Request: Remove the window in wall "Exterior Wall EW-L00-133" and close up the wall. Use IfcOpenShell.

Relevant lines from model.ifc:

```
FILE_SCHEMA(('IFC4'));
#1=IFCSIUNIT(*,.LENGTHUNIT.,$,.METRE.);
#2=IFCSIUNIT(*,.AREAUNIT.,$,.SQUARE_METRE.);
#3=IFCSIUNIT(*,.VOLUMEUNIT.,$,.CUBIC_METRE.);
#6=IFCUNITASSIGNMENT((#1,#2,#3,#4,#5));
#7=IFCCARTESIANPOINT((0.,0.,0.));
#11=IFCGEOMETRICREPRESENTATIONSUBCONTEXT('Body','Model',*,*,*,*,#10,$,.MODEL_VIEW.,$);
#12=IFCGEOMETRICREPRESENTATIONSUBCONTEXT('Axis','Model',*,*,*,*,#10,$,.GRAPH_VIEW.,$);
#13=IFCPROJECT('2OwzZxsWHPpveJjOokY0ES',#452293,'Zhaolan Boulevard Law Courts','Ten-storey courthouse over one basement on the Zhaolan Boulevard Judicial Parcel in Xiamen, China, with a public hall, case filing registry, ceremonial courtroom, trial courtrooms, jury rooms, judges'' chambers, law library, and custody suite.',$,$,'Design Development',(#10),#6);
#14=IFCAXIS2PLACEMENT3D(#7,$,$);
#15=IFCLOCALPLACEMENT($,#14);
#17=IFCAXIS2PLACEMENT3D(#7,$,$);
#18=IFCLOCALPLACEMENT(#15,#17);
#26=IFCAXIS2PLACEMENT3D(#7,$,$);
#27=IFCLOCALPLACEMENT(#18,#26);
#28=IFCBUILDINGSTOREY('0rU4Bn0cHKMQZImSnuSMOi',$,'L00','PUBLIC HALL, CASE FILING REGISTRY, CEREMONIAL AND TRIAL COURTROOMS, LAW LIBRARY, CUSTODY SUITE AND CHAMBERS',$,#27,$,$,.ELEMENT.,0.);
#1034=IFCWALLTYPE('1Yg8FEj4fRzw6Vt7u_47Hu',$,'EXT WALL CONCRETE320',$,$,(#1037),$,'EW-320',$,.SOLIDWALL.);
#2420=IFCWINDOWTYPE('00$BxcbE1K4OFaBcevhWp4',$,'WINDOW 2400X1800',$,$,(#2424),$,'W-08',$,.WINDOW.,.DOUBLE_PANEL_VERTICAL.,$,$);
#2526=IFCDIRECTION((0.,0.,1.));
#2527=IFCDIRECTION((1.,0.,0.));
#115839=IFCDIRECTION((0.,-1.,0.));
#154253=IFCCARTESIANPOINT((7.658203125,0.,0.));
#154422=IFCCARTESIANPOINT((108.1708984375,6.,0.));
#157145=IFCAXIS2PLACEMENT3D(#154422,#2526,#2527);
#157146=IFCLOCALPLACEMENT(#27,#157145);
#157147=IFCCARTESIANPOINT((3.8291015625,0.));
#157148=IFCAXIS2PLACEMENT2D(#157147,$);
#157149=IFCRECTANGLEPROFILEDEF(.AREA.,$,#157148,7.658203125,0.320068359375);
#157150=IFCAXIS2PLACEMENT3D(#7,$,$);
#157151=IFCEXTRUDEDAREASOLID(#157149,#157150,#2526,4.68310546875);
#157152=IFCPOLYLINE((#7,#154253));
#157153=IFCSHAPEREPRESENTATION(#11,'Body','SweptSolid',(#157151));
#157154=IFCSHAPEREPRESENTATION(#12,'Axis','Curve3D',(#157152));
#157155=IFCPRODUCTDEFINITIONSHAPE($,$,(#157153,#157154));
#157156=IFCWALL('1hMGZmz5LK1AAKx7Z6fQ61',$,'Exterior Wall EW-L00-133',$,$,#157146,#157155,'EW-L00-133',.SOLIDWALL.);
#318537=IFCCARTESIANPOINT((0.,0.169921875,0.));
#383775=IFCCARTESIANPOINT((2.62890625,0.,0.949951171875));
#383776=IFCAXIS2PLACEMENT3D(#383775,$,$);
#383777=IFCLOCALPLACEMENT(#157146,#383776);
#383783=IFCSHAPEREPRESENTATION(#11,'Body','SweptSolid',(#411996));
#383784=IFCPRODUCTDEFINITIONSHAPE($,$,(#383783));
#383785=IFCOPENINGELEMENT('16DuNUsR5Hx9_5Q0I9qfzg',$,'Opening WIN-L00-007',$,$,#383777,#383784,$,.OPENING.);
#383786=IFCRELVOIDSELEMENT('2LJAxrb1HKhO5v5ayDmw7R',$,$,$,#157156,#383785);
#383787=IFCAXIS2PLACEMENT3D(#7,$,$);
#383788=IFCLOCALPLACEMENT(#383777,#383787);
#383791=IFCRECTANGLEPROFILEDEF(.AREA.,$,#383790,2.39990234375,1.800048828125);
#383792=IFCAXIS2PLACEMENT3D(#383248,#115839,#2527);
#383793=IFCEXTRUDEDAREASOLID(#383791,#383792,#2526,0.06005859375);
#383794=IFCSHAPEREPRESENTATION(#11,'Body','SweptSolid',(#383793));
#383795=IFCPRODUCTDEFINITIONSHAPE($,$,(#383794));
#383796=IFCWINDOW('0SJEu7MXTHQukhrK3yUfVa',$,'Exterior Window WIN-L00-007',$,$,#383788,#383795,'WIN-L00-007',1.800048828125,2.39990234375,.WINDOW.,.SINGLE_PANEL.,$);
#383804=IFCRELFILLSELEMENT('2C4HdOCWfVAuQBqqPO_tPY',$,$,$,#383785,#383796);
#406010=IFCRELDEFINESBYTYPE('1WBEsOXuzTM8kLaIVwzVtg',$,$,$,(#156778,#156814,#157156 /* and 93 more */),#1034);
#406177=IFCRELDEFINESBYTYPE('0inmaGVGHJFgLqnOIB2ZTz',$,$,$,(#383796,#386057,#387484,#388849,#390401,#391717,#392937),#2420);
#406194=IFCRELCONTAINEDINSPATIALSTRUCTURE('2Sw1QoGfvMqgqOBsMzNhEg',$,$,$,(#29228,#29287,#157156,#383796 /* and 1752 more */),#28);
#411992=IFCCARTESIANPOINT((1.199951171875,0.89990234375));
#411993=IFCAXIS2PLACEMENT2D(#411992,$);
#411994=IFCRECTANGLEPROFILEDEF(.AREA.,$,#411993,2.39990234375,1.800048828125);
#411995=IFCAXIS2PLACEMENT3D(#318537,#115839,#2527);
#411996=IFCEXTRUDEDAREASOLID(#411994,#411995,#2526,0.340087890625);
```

```python
import ifcopenshell
import ifcopenshell.api.feature
import ifcopenshell.api.root
import ifcopenshell.geom
import ifcopenshell.util.shape

model = ifcopenshell.open("model.ifc")
settings = ifcopenshell.geom.settings()


def volume(element):
    """Net volume in cubic metres, openings subtracted."""
    shape = ifcopenshell.geom.create_shape(settings, element)
    return ifcopenshell.util.shape.get_volume(shape.geometry)


window = model.by_guid("0SJEu7MXTHQukhrK3yUfVa")
opening = window.FillsVoids[0].RelatingOpeningElement
wall = opening.VoidsElements[0].RelatingBuildingElement
before = volume(wall)

ifcopenshell.api.root.remove_product(model, product=window)
ifcopenshell.api.feature.remove_feature(model, feature=opening)

after = volume(wall)

print(f"wall volume {before:.3f} -> {after:.3f} m3")

model.write("model_updated.ifc")
```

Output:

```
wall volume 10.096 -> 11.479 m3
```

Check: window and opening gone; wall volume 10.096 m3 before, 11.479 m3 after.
